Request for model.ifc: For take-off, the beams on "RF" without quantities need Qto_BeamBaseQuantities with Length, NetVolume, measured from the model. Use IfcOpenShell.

First a look at what the model holds.

```python
import ifcopenshell
import ifcopenshell.util.element
import ifcopenshell.util.unit

model = ifcopenshell.open("model.ifc")
print(model.schema)
for unit_type in ("LENGTHUNIT", "AREAUNIT", "VOLUMEUNIT"):
    print(unit_type, ifcopenshell.util.unit.calculate_unit_scale(model, unit_type))
storey = next(s for s in model.by_type("IfcBuildingStorey") if s.Name == "RF")
beams = [e for e in ifcopenshell.util.element.get_decomposition(storey) if e.is_a("IfcBeam")]
for e in sorted(beams, key=lambda e: e.id()):
    print(e.id(), e.is_a(), e.Name, list(ifcopenshell.util.element.get_psets(e, qtos_only=True)), sep=" | ")
```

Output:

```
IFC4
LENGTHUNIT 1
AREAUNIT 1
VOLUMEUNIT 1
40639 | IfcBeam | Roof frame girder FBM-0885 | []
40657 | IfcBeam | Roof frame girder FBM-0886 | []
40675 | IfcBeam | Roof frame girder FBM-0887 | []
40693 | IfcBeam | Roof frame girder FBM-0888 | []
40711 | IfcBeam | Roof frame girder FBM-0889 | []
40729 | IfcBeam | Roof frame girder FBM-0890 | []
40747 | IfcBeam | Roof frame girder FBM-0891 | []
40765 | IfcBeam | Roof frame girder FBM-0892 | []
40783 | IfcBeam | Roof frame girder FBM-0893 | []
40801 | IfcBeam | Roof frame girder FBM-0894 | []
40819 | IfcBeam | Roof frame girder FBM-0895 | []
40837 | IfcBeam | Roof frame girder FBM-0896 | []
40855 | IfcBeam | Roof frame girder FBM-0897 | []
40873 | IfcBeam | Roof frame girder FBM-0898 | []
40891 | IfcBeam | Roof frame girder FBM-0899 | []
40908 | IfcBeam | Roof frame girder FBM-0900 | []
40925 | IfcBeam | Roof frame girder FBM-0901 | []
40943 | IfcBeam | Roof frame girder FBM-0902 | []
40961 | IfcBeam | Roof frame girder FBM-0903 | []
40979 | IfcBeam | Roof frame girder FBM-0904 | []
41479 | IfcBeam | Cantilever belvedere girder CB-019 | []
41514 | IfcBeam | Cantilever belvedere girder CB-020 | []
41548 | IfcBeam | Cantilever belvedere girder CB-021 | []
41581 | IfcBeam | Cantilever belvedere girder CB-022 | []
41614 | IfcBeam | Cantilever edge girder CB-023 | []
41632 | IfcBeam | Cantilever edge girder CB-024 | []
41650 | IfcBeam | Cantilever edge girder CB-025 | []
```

```python
import ifcopenshell
import ifcopenshell.api.pset
import ifcopenshell.geom
import ifcopenshell.util.element
import ifcopenshell.util.shape
import ifcopenshell.util.unit

model = ifcopenshell.open("model.ifc")
unit_scale = ifcopenshell.util.unit.calculate_unit_scale(model)
volume_scale = ifcopenshell.util.unit.calculate_unit_scale(model, "VOLUMEUNIT")
settings = ifcopenshell.geom.settings()

storey = next(s for s in model.by_type("IfcBuildingStorey") if s.Name == "RF")
beams = [e for e in ifcopenshell.util.element.get_decomposition(storey) if e.is_a("IfcBeam")]

for e in sorted(beams, key=lambda e: e.id()):
    if ifcopenshell.util.element.get_psets(e, qtos_only=True, should_inherit=False):
        continue
    # Geometry comes back in metres, in the element's own axes.
    shape = ifcopenshell.geom.create_shape(settings, e)
    values = {
        "Length": ifcopenshell.util.shape.get_max_xyz(shape.geometry) / unit_scale,
        "NetVolume": ifcopenshell.util.shape.get_volume(shape.geometry) / volume_scale,
    }
    qto = ifcopenshell.api.pset.add_qto(model, product=e, name="Qto_BeamBaseQuantities")
    ifcopenshell.api.pset.edit_qto(model, qto=qto, properties=values)
    print(e.id(), {k: round(v, 3) for k, v in values.items()})

model.write("model-out.ifc")
```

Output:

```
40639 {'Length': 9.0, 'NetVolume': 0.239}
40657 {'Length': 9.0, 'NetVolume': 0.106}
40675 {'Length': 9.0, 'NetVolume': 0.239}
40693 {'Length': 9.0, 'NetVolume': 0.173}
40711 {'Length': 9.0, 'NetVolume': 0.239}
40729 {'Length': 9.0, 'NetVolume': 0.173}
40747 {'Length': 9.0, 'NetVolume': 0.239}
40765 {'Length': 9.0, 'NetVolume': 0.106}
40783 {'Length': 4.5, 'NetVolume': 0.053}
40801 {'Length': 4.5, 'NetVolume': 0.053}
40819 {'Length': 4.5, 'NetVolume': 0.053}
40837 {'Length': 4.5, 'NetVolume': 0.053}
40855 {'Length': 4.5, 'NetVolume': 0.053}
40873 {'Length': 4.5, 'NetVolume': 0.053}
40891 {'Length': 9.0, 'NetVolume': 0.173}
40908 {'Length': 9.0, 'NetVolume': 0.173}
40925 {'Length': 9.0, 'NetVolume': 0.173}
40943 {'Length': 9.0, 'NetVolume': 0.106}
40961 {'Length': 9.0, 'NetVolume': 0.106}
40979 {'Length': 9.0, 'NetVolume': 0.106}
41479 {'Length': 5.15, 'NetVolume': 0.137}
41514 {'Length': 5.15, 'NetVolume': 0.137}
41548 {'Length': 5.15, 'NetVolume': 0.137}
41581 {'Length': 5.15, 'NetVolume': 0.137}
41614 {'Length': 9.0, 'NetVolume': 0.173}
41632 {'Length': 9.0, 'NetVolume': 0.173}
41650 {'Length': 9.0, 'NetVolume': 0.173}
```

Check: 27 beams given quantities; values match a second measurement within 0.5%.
